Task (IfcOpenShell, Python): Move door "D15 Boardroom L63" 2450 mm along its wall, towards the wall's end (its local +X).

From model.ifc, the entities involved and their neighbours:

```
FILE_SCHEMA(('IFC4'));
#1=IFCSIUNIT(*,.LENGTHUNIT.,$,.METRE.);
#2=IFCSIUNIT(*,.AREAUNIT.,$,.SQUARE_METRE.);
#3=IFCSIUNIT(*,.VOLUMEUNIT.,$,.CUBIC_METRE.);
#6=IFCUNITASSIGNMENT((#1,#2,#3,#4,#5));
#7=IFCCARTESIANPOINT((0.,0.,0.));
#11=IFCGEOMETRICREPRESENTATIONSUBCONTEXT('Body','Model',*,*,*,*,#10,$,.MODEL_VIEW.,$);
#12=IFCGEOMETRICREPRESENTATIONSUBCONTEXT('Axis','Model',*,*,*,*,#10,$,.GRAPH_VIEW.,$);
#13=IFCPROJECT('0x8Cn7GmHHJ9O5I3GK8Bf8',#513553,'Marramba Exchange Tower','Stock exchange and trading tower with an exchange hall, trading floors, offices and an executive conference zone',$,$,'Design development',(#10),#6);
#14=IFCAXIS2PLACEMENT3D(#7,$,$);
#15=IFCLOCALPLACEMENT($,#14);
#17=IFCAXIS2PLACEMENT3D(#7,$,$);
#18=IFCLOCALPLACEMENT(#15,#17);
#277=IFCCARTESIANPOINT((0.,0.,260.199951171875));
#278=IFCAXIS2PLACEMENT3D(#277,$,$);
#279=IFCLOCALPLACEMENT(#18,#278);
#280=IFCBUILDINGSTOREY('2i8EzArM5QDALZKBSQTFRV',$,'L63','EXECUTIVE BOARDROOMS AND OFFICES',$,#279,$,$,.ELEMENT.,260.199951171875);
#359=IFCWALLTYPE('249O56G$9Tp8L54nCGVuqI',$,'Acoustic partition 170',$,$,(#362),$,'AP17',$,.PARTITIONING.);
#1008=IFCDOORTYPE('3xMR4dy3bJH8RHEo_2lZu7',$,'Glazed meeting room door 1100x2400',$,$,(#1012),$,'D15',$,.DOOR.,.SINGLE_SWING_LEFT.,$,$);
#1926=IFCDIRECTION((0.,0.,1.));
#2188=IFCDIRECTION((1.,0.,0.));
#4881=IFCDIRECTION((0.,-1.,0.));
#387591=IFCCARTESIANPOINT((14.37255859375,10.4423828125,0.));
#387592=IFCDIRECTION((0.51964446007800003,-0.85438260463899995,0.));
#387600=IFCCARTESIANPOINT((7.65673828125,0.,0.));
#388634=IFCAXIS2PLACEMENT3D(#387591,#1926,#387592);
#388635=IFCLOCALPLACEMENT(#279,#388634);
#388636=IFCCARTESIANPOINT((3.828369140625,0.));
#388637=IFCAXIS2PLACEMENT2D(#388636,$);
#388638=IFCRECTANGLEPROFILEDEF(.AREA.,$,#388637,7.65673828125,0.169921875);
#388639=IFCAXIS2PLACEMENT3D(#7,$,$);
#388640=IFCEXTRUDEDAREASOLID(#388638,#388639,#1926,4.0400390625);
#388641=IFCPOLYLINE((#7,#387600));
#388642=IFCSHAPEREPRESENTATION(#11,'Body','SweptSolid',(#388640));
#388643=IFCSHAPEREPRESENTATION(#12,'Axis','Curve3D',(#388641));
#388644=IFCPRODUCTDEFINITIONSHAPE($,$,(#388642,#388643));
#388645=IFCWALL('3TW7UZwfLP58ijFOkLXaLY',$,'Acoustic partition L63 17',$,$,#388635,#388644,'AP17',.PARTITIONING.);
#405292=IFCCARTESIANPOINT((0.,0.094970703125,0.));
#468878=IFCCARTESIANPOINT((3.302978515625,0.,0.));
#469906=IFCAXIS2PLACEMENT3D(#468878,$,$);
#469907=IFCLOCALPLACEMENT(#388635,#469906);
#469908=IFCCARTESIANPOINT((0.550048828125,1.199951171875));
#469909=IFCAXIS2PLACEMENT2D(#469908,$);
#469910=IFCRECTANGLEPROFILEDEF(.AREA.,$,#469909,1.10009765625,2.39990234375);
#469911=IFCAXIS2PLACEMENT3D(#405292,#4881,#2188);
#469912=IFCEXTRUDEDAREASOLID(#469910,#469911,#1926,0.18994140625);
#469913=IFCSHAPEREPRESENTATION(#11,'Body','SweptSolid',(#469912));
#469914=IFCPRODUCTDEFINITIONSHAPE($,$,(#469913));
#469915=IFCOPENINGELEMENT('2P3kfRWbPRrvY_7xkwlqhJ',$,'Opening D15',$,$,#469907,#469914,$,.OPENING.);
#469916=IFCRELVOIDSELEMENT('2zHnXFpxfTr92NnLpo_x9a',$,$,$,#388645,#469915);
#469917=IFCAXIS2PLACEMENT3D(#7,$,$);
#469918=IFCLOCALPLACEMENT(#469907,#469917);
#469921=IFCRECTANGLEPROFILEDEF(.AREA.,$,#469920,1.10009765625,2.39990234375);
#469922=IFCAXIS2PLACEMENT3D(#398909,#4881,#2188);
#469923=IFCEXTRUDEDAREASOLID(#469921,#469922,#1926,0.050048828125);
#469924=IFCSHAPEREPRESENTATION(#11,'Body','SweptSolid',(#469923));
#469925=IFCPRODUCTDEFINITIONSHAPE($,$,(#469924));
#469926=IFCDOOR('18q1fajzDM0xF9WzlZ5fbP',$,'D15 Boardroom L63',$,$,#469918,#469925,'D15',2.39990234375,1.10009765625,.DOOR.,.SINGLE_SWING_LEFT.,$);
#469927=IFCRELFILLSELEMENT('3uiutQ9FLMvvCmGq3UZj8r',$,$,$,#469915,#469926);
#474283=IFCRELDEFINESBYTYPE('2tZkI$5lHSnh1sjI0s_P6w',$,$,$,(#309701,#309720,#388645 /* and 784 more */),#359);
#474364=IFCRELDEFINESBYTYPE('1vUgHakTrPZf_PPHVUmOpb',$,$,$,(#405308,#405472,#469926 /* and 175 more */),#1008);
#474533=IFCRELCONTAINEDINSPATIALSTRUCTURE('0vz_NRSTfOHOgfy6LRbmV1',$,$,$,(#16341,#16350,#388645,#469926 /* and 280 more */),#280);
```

```python
import ifcopenshell
import ifcopenshell.api.geometry
import ifcopenshell.util.placement
import ifcopenshell.util.unit

model = ifcopenshell.open("model.ifc")
unit_scale = ifcopenshell.util.unit.calculate_unit_scale(model)

door = model.by_guid("18q1fajzDM0xF9WzlZ5fbP")
opening = door.FillsVoids[0].RelatingOpeningElement
wall = opening.VoidsElements[0].RelatingBuildingElement

wall_matrix = ifcopenshell.util.placement.get_local_placement(wall.ObjectPlacement)
shift = wall_matrix[:3, 0] * 2.45 / unit_scale
before = ifcopenshell.util.placement.get_local_placement(door.ObjectPlacement)[:3, 3].copy()

# The door is placed relative to its opening, so it follows when the opening moves.
matrix = ifcopenshell.util.placement.get_local_placement(opening.ObjectPlacement)
matrix[:3, 3] += shift
ifcopenshell.api.geometry.edit_object_placement(
    model, product=opening, matrix=matrix, is_si=False, should_transform_children=True
)

after = ifcopenshell.util.placement.get_local_placement(door.ObjectPlacement)[:3, 3]
print("door moved by", (after - before).round(3) + 0.0)

model.write("model_v2.ifc")
```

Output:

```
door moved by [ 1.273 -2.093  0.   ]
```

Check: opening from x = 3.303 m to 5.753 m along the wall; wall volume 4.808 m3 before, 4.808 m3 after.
